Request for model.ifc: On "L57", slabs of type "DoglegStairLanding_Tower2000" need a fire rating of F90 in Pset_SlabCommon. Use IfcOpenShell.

First a look at what the model holds.

```python
import ifcopenshell
import ifcopenshell.util.element

model = ifcopenshell.open("model.ifc")
print(model.schema)
storey = next(s for s in model.by_type("IfcBuildingStorey") if s.Name == "L57")
slabs = [e for e in ifcopenshell.util.element.get_decomposition(storey) if e.is_a("IfcSlab")]
seen = {}
for e in slabs:
    element_type = ifcopenshell.util.element.get_type(e)
    key = (element_type.Name if element_type != e and element_type else None, ifcopenshell.util.element.get_pset(e, "Pset_SlabCommon", "FireRating"))
    seen[key] = seen.get(key, 0) + 1
for (name, value), count in sorted(seen.items(), key=str):
    print(count, "x", name, "|", value)
```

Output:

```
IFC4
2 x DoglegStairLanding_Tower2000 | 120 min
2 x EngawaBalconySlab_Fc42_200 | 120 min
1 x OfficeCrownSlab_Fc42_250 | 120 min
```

```python
import ifcopenshell
import ifcopenshell.api.pset
import ifcopenshell.util.element

model = ifcopenshell.open("model.ifc")

storey = next(s for s in model.by_type("IfcBuildingStorey") if s.Name == "L57")
slabs = [e for e in ifcopenshell.util.element.get_decomposition(storey) if e.is_a("IfcSlab")]

count = 0
for e in slabs:
    element_type = ifcopenshell.util.element.get_type(e)
    if element_type in (None, e) or element_type.Name != "DoglegStairLanding_Tower2000":
        continue
    # add_pset returns the element's existing set when there is one.
    pset = ifcopenshell.api.pset.add_pset(model, product=e, name="Pset_SlabCommon")
    ifcopenshell.api.pset.edit_pset(model, pset=pset, properties={"FireRating": "F90"})
    count += 1

print(count, "slabs updated")

model.write("model_v2.ifc")
```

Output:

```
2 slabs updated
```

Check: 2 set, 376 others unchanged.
